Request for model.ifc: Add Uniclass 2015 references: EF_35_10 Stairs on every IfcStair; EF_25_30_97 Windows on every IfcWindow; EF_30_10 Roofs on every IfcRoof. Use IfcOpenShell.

First a look at what the model holds.

```python
import ifcopenshell

model = ifcopenshell.open("model.ifc")
print(model.schema)
print("classifications:", [c.Name for c in model.by_type("IfcClassification")])
for ifc_class in ("IfcDoor", "IfcRoof", "IfcStair", "IfcWall", "IfcWindow"):
    print(ifc_class, len(model.by_type(ifc_class)))
```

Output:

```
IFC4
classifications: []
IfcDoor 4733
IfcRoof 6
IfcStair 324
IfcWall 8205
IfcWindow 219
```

```python
import ifcopenshell
import ifcopenshell.api.classification

model = ifcopenshell.open("model.ifc")

system = ifcopenshell.api.classification.add_classification(model, classification="Uniclass 2015")

codes = {
    "IfcStair": ("EF_35_10", "Stairs"),
    "IfcWindow": ("EF_25_30_97", "Windows"),
    "IfcRoof": ("EF_30_10", "Roofs"),
}
for ifc_class, (code, name) in codes.items():
    products = model.by_type(ifc_class)
    ifcopenshell.api.classification.add_reference(
        model, products=products, classification=system, identification=code, name=name
    )
    print(code, len(products))

model.write("model_updated.ifc")
```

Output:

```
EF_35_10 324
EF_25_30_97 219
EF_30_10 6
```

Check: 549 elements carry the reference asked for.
